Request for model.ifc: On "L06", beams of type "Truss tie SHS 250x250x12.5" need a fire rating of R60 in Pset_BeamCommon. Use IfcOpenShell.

First a look at what the model holds.

```python
import ifcopenshell
import ifcopenshell.util.element

model = ifcopenshell.open("model.ifc")
print(model.schema)
storey = next(s for s in model.by_type("IfcBuildingStorey") if s.Name == "L06")
beams = [e for e in ifcopenshell.util.element.get_decomposition(storey) if e.is_a("IfcBeam")]
seen = {}
for e in beams:
    element_type = ifcopenshell.util.element.get_type(e)
    key = (element_type.Name if element_type != e and element_type else None, ifcopenshell.util.element.get_pset(e, "Pset_BeamCommon", "FireRating"))
    seen[key] = seen.get(key, 0) + 1
for (name, value), count in sorted(seen.items(), key=str):
    print(count, "x", name, "|", value)
```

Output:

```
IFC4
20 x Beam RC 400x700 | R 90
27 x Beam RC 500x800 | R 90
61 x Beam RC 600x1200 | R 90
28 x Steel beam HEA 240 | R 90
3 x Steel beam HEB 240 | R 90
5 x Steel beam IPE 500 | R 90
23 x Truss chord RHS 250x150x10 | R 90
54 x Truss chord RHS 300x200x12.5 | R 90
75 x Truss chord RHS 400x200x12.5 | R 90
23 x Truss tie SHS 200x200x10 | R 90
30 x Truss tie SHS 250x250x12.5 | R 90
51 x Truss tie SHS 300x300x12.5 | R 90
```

```python
import ifcopenshell
import ifcopenshell.api.pset
import ifcopenshell.util.element

model = ifcopenshell.open("model.ifc")

storey = next(s for s in model.by_type("IfcBuildingStorey") if s.Name == "L06")
beams = [e for e in ifcopenshell.util.element.get_decomposition(storey) if e.is_a("IfcBeam")]

count = 0
for e in beams:
    element_type = ifcopenshell.util.element.get_type(e)
    if element_type in (None, e) or element_type.Name != "Truss tie SHS 250x250x12.5":
        continue
    # add_pset returns the element's existing set when there is one.
    pset = ifcopenshell.api.pset.add_pset(model, product=e, name="Pset_BeamCommon")
    ifcopenshell.api.pset.edit_pset(model, pset=pset, properties={"FireRating": "R60"})
    count += 1

print(count, "beams updated")

model.write("model_edited.ifc")
```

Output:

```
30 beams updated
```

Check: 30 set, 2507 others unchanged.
